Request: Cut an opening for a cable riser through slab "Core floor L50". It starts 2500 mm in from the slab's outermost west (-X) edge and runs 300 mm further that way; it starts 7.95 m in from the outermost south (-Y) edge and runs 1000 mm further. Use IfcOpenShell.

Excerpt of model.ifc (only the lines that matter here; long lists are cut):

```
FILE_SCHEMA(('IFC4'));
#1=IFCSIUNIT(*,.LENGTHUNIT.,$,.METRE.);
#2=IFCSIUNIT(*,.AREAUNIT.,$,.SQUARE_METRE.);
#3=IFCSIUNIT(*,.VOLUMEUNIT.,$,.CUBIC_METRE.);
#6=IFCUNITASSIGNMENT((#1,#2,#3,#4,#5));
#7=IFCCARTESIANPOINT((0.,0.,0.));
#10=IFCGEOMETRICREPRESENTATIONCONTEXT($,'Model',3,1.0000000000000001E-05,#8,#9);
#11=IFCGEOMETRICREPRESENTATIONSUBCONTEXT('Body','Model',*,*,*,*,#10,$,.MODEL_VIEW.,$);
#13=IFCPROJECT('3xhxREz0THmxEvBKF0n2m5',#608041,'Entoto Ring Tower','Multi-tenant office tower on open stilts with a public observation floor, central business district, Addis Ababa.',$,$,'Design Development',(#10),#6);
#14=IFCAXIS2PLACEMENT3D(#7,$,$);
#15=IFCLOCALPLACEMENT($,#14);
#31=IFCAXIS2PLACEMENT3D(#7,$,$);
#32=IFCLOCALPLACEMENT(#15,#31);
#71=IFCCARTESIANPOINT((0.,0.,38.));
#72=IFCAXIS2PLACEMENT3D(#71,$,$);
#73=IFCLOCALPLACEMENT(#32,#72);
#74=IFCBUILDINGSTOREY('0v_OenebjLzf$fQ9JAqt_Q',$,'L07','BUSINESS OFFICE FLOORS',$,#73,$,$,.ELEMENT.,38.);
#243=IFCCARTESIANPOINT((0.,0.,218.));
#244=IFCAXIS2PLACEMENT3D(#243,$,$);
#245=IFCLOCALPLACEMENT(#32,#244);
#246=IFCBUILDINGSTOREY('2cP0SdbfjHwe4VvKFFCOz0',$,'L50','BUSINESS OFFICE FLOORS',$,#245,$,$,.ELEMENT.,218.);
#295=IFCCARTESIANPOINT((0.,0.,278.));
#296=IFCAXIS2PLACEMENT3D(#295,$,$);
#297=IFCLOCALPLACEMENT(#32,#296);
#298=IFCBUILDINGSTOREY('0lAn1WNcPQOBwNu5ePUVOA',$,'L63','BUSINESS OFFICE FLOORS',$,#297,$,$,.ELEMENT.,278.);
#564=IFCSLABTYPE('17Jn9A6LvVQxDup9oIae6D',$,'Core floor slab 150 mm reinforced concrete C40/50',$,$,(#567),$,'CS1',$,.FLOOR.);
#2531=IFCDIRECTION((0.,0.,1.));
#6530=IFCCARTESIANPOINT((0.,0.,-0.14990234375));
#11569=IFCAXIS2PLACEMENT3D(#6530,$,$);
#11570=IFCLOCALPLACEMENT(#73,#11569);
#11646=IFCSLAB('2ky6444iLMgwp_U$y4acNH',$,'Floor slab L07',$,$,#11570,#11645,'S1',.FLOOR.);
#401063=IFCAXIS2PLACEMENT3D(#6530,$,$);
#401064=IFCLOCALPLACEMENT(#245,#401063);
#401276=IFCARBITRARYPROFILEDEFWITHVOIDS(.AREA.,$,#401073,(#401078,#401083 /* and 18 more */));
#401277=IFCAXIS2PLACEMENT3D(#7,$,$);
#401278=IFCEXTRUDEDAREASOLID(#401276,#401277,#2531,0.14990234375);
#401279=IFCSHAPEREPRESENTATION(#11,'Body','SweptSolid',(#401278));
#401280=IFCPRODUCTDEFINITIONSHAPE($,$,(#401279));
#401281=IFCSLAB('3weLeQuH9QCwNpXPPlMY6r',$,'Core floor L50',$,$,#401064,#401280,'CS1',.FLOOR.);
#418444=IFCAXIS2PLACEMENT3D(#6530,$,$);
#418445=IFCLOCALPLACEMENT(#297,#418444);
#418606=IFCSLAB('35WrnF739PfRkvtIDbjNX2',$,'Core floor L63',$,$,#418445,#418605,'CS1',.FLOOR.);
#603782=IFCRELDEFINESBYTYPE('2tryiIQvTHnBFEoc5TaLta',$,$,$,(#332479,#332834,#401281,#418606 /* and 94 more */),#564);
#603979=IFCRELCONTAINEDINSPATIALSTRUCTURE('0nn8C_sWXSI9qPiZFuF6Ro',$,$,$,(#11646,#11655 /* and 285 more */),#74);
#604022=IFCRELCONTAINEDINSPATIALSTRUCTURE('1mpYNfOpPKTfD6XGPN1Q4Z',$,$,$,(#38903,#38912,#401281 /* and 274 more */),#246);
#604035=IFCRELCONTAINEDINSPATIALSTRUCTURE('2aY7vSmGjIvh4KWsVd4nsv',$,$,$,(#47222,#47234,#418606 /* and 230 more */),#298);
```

```python
import numpy as np
import ifcopenshell
import ifcopenshell.api.feature
import ifcopenshell.api.geometry
import ifcopenshell.api.root
import ifcopenshell.geom
import ifcopenshell.util.placement
import ifcopenshell.util.representation
import ifcopenshell.util.shape
import ifcopenshell.util.unit

model = ifcopenshell.open("model.ifc")
unit_scale = ifcopenshell.util.unit.calculate_unit_scale(model)
settings = ifcopenshell.geom.settings()


def volume(element):
    """Net volume in cubic metres, openings subtracted."""
    shape = ifcopenshell.geom.create_shape(settings, element)
    return ifcopenshell.util.shape.get_volume(shape.geometry)


slab = model.by_guid("3weLeQuH9QCwNpXPPlMY6r")
before = volume(slab)

# Extent in the slab's own axes, in metres. The edges named are its -X and -Y sides.
slab_shape = ifcopenshell.geom.create_shape(settings, slab)
vertices = ifcopenshell.util.shape.get_vertices(slab_shape.geometry)
x_min, y_min, bottom = vertices.min(axis=0)
top = vertices[:, 2].max()

opening = ifcopenshell.api.root.create_entity(model, ifc_class="IfcOpeningElement", name="Cable riser opening", predefined_type="OPENING")
context = ifcopenshell.util.representation.get_context(model, "Model", "Body", "MODEL_VIEW")
width, depth = 0.3, 1
outline = [(0.0, 0.0), (width, 0.0), (width, depth), (0.0, depth), (0.0, 0.0)]
# Overshoot both faces by 50 mm so the cut is clean.
shape = ifcopenshell.api.geometry.add_slab_representation(
    model, context=context, depth=top - bottom + 0.1, polyline=outline
)
ifcopenshell.api.geometry.assign_representation(model, product=opening, representation=shape)

matrix = ifcopenshell.util.placement.get_local_placement(slab.ObjectPlacement)
matrix[:, 3] = matrix @ np.append(np.array([x_min + 2.5, y_min + 7.95, bottom - 0.05]) / unit_scale, 1.0)
ifcopenshell.api.geometry.edit_object_placement(model, product=opening, matrix=matrix, is_si=False)
ifcopenshell.api.feature.add_feature(model, feature=opening, element=slab)

after = volume(slab)

print(f"slab volume {before:.3f} -> {after:.3f} m3")

model.write("model-out.ifc")
```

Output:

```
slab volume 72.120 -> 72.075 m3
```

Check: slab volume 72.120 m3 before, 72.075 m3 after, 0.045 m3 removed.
